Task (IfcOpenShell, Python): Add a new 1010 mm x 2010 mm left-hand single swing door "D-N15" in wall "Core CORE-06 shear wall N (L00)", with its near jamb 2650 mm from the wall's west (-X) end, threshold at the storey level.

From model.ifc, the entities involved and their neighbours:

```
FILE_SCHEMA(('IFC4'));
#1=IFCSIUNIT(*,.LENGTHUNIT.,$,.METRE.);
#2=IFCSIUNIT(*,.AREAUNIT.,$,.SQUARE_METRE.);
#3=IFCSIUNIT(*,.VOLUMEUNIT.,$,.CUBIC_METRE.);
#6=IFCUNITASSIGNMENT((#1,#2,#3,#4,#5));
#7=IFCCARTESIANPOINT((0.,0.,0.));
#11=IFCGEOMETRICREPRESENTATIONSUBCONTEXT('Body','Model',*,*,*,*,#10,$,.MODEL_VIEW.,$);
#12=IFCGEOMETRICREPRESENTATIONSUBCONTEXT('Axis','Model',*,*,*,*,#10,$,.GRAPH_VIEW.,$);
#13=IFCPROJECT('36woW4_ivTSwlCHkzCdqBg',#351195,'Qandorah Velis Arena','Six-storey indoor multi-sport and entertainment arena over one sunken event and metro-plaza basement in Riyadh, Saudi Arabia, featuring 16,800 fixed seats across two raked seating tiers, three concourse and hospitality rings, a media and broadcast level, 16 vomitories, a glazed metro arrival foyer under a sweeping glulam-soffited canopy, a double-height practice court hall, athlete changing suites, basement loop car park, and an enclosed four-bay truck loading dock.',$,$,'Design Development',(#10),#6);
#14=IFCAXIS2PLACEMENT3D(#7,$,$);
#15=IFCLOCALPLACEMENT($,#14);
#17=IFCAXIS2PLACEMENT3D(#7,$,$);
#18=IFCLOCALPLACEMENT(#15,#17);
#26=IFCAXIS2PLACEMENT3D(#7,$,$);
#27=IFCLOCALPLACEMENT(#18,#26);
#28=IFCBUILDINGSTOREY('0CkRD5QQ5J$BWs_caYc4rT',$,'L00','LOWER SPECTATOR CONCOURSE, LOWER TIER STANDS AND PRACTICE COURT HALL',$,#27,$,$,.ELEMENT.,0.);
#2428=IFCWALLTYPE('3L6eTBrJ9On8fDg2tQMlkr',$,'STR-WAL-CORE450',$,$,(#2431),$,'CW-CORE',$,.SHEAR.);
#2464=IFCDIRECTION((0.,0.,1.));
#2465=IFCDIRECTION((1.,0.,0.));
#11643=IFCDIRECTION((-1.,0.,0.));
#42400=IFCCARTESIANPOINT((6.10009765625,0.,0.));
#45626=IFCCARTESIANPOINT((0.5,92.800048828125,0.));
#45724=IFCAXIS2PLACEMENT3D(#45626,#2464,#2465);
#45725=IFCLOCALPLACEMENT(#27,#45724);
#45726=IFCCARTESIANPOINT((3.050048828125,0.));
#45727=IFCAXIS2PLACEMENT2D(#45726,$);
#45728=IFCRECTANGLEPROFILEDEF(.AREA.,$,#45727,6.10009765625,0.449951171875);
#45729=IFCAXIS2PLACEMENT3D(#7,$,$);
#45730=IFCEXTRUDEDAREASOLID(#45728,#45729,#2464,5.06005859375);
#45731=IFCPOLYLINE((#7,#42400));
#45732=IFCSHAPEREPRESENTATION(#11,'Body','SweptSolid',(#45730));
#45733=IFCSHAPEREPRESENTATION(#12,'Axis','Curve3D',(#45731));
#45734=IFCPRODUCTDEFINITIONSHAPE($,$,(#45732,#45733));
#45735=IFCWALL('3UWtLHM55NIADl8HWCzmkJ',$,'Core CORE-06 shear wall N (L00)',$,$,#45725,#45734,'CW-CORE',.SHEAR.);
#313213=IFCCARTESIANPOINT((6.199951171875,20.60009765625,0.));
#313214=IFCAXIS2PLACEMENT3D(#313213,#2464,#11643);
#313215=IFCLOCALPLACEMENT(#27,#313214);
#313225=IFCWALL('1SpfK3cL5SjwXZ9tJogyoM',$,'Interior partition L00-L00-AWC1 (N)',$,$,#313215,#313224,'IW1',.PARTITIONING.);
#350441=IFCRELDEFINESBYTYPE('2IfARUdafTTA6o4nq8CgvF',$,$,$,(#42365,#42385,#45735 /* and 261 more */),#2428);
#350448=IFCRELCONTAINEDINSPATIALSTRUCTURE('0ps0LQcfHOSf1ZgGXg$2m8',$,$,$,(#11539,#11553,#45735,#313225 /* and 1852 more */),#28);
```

```python
import numpy as np
import ifcopenshell
import ifcopenshell.api.feature
import ifcopenshell.api.geometry
import ifcopenshell.api.root
import ifcopenshell.api.spatial
import ifcopenshell.geom
import ifcopenshell.util.element
import ifcopenshell.util.placement
import ifcopenshell.util.representation
import ifcopenshell.util.shape
import ifcopenshell.util.unit

model = ifcopenshell.open("model.ifc")
unit_scale = ifcopenshell.util.unit.calculate_unit_scale(model)
settings = ifcopenshell.geom.settings()


def volume(element):
    """Net volume in cubic metres, openings subtracted."""
    shape = ifcopenshell.geom.create_shape(settings, element)
    return ifcopenshell.util.shape.get_volume(shape.geometry)


wall = model.by_guid("3UWtLHM55NIADl8HWCzmkJ")
storey = ifcopenshell.util.element.get_container(wall, ifc_class="IfcBuildingStorey")
context = ifcopenshell.util.representation.get_context(model, "Model", "Body", "MODEL_VIEW")
before = volume(wall)

width, height, from_end, sill = 1.01, 2.01, 2.65, 0.0  # metres

# The wall runs along its own X axis, and the end named is its -X end.
wall_shape = ifcopenshell.geom.create_shape(settings, wall)
x, y, z = ifcopenshell.util.shape.get_vertices(wall_shape.geometry).T
start = x.min() + from_end
face, thickness = float(y.min()), float(y.max() - y.min())
wall_matrix = ifcopenshell.util.placement.get_local_placement(wall.ObjectPlacement)
level = ifcopenshell.util.placement.get_local_placement(storey.ObjectPlacement)[2, 3]


def in_wall(x, y):
    """Placement at x, y metres in the wall's axes, at sill height."""
    matrix = wall_matrix.copy()
    matrix[:, 3] = wall_matrix @ np.array([x / unit_scale, y / unit_scale, 0.0, 1.0])
    matrix[2, 3] = level + sill / unit_scale
    return matrix


# Opening: a box that overshoots both wall faces by 50 mm.
opening = ifcopenshell.api.root.create_entity(model, ifc_class="IfcOpeningElement", predefined_type="OPENING")
box = ifcopenshell.api.geometry.add_wall_representation(
    model, context=context, length=width, height=height, thickness=thickness + 0.1
)
ifcopenshell.api.geometry.assign_representation(model, product=opening, representation=box)
ifcopenshell.api.geometry.edit_object_placement(model, product=opening, matrix=in_wall(start, face - 0.05), is_si=False)
ifcopenshell.api.feature.add_feature(model, feature=opening, element=wall)

door = ifcopenshell.api.root.create_entity(model, ifc_class="IfcDoor", name="D-N15", predefined_type="DOOR")
door.OverallWidth, door.OverallHeight = width / unit_scale, height / unit_scale
door.OperationType = "SINGLE_SWING_LEFT"
body = ifcopenshell.api.geometry.add_door_representation(
    model,
    context=context,
    overall_width=door.OverallWidth,
    overall_height=door.OverallHeight,
    operation_type="SINGLE_SWING_LEFT",
    lining_properties={"LiningDepth": thickness / unit_scale, "ThresholdDepth": thickness / unit_scale},
)
ifcopenshell.api.geometry.assign_representation(model, product=door, representation=body)
ifcopenshell.api.spatial.assign_container(model, products=[door], relating_structure=storey)
ifcopenshell.api.feature.add_filling(model, opening=opening, element=door)

# The lining spans the wall, so the door starts at the wall face.
ifcopenshell.api.geometry.edit_object_placement(model, product=door, matrix=in_wall(start, face), is_si=False)

after = volume(wall)

print(f"wall volume {before:.3f} -> {after:.3f} m3")

model.write("model_edited.ifc")
```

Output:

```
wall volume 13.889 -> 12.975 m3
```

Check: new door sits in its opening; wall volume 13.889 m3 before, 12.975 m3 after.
